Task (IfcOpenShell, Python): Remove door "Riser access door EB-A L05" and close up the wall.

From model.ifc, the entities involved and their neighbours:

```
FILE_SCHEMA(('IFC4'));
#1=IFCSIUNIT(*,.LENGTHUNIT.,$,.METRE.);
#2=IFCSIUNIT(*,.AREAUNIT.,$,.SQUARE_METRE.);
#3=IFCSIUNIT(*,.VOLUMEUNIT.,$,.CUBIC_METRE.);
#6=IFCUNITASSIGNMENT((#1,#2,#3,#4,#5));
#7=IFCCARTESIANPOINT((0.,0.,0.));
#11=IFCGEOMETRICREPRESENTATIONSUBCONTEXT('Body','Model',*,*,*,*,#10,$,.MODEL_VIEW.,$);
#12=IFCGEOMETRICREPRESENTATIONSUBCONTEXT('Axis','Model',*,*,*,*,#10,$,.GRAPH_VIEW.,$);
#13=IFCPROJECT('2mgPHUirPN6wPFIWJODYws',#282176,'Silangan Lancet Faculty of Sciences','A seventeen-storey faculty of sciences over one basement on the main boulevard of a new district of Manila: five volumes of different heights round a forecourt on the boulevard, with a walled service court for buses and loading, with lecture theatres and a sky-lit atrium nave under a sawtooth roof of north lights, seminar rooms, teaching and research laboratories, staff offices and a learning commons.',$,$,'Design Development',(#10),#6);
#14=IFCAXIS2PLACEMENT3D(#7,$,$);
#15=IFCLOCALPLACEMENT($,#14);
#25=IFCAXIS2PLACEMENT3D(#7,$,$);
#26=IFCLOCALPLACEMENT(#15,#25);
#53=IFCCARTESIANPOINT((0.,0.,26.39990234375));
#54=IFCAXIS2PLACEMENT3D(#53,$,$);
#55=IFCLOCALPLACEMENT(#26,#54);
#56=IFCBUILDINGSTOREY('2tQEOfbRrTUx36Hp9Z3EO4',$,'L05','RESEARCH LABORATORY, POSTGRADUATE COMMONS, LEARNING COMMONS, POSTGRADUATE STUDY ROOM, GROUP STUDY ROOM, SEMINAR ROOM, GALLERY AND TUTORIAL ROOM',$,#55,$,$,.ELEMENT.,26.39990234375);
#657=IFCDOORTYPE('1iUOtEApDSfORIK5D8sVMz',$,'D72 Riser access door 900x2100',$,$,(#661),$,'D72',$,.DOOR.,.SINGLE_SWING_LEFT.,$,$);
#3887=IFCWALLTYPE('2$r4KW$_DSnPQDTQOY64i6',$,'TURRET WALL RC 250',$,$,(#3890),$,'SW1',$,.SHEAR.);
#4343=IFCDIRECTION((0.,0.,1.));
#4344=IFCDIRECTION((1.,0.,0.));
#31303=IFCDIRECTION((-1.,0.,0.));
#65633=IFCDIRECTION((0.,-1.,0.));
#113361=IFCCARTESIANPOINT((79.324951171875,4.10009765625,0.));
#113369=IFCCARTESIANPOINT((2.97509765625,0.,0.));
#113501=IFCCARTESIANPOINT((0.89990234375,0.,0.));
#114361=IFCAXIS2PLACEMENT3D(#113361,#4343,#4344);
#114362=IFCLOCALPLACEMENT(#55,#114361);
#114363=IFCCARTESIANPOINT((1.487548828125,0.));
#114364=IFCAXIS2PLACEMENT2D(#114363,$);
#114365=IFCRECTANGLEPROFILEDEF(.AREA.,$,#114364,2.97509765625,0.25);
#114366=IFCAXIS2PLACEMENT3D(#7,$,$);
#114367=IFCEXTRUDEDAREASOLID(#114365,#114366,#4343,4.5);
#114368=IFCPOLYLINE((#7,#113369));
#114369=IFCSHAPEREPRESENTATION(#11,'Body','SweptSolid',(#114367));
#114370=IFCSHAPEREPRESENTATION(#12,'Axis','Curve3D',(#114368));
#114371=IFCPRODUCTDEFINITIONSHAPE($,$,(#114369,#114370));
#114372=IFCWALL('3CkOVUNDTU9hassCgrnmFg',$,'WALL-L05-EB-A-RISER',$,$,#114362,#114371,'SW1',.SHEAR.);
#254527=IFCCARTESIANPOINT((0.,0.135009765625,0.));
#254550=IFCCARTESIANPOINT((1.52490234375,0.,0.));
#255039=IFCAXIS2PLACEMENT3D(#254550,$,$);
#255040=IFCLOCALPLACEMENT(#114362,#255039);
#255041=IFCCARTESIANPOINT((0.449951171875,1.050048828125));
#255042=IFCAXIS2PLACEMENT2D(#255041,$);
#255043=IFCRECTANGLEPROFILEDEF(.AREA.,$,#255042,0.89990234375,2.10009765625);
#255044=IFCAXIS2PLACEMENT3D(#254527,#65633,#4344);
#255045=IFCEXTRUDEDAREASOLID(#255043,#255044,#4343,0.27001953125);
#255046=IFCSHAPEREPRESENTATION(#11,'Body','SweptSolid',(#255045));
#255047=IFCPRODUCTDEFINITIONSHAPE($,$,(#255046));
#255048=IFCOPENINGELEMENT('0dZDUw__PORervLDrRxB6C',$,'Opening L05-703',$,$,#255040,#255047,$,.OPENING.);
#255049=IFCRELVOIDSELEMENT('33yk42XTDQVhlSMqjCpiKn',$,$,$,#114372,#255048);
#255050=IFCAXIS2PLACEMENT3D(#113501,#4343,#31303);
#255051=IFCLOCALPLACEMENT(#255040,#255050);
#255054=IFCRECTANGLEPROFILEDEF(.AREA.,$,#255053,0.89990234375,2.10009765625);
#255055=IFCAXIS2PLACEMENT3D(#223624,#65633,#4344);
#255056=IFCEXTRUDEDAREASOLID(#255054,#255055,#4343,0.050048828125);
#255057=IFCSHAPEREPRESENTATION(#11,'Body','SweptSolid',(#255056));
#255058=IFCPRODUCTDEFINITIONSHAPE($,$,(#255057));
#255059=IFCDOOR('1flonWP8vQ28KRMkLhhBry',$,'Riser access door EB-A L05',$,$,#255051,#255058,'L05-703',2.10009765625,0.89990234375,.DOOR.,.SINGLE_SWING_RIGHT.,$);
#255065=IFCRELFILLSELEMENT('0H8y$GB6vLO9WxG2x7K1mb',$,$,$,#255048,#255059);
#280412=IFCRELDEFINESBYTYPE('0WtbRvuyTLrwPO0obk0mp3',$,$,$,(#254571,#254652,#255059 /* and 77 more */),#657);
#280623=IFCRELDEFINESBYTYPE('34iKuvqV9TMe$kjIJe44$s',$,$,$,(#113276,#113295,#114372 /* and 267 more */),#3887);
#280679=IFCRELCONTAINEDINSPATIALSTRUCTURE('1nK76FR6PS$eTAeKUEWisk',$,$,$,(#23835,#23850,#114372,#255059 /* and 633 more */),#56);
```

```python
import ifcopenshell
import ifcopenshell.api.feature
import ifcopenshell.api.root
import ifcopenshell.geom
import ifcopenshell.util.shape

model = ifcopenshell.open("model.ifc")
settings = ifcopenshell.geom.settings()


def volume(element):
    """Net volume in cubic metres, openings subtracted."""
    shape = ifcopenshell.geom.create_shape(settings, element)
    return ifcopenshell.util.shape.get_volume(shape.geometry)


door = model.by_guid("1flonWP8vQ28KRMkLhhBry")
opening = door.FillsVoids[0].RelatingOpeningElement
wall = opening.VoidsElements[0].RelatingBuildingElement
before = volume(wall)

ifcopenshell.api.root.remove_product(model, product=door)
ifcopenshell.api.feature.remove_feature(model, feature=opening)

after = volume(wall)

print(f"wall volume {before:.3f} -> {after:.3f} m3")

model.write("model_updated.ifc")
```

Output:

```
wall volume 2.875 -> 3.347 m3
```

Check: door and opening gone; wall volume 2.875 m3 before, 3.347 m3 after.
